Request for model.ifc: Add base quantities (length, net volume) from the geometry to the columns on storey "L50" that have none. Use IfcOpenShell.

First a look at what the model holds.

```python
import ifcopenshell
import ifcopenshell.util.element
import ifcopenshell.util.unit

model = ifcopenshell.open("model.ifc")
print(model.schema)
for unit_type in ("LENGTHUNIT", "AREAUNIT", "VOLUMEUNIT"):
    print(unit_type, ifcopenshell.util.unit.calculate_unit_scale(model, unit_type))
storey = next(s for s in model.by_type("IfcBuildingStorey") if s.Name == "L50")
columns = [e for e in ifcopenshell.util.element.get_decomposition(storey) if e.is_a("IfcColumn")]
for e in sorted(columns, key=lambda e: e.id()):
    print(e.id(), e.is_a(), e.Name, list(ifcopenshell.util.element.get_psets(e, qtos_only=True)), sep=" | ")
```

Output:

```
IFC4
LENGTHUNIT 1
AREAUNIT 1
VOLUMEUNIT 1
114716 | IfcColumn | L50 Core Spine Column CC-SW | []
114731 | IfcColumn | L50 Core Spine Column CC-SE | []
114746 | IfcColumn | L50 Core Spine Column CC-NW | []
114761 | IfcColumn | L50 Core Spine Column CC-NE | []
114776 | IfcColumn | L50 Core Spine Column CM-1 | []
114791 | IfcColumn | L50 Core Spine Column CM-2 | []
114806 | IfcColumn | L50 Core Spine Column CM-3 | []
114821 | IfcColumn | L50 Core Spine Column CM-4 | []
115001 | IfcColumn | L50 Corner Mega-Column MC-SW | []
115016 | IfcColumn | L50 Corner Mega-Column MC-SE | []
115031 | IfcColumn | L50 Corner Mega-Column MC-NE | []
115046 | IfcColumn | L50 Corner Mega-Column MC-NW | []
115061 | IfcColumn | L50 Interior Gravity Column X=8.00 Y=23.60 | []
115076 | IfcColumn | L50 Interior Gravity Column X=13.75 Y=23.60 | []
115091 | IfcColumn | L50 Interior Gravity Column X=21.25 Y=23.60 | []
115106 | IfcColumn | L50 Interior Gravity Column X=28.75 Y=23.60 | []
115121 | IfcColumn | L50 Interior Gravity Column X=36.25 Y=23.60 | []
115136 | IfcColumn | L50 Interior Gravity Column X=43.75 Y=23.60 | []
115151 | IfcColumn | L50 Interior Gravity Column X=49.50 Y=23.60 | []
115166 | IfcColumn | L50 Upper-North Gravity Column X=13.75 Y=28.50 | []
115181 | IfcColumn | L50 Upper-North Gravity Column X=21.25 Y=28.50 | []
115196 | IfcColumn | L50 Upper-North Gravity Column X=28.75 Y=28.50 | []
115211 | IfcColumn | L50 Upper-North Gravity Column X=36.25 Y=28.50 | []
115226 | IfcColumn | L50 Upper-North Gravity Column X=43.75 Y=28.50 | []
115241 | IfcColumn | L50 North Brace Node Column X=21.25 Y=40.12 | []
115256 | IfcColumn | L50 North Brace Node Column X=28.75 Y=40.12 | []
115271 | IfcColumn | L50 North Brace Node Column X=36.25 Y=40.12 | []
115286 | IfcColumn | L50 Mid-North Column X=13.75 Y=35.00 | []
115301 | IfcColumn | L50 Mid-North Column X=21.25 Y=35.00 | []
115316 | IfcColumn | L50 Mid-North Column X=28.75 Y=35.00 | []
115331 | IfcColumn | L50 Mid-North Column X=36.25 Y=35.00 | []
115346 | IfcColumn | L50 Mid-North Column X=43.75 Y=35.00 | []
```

```python
import ifcopenshell
import ifcopenshell.api.pset
import ifcopenshell.geom
import ifcopenshell.util.element
import ifcopenshell.util.shape
import ifcopenshell.util.unit

model = ifcopenshell.open("model.ifc")
unit_scale = ifcopenshell.util.unit.calculate_unit_scale(model)
volume_scale = ifcopenshell.util.unit.calculate_unit_scale(model, "VOLUMEUNIT")
settings = ifcopenshell.geom.settings()

storey = next(s for s in model.by_type("IfcBuildingStorey") if s.Name == "L50")
columns = [e for e in ifcopenshell.util.element.get_decomposition(storey) if e.is_a("IfcColumn")]

for e in sorted(columns, key=lambda e: e.id()):
    if ifcopenshell.util.element.get_psets(e, qtos_only=True, should_inherit=False):
        continue
    # Geometry comes back in metres, in the element's own axes.
    shape = ifcopenshell.geom.create_shape(settings, e)
    values = {
        "Length": ifcopenshell.util.shape.get_z(shape.geometry) / unit_scale,
        "NetVolume": ifcopenshell.util.shape.get_volume(shape.geometry) / volume_scale,
    }
    qto = ifcopenshell.api.pset.add_qto(model, product=e, name="Qto_ColumnBaseQuantities")
    ifcopenshell.api.pset.edit_qto(model, qto=qto, properties=values)
    print(e.id(), {k: round(v, 3) for k, v in values.items()})

model.write("model_v2.ifc")
```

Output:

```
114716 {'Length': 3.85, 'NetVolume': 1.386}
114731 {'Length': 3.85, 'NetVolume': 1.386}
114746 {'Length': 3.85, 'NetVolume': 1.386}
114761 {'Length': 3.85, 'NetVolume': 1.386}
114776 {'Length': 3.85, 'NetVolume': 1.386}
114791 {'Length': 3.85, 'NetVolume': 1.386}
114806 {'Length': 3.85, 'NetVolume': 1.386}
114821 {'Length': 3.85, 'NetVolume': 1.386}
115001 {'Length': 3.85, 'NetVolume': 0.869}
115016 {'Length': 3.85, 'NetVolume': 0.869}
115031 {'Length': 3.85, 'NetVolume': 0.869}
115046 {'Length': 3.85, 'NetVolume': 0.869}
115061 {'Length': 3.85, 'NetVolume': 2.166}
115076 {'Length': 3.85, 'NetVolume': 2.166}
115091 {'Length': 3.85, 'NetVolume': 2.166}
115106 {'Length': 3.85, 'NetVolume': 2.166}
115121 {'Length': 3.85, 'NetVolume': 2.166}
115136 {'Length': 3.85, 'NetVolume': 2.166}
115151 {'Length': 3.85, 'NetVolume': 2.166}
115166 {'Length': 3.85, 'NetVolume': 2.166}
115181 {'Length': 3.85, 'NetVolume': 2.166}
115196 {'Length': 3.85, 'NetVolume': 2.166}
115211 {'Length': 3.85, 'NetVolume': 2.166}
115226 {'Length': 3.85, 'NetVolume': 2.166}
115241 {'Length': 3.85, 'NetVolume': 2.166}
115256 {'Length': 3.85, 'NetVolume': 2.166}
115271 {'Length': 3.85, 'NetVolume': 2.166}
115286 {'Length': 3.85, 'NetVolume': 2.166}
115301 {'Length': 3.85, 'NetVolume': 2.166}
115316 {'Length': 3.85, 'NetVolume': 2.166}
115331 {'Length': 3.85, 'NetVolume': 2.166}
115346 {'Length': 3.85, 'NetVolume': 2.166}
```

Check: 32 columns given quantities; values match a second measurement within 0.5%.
